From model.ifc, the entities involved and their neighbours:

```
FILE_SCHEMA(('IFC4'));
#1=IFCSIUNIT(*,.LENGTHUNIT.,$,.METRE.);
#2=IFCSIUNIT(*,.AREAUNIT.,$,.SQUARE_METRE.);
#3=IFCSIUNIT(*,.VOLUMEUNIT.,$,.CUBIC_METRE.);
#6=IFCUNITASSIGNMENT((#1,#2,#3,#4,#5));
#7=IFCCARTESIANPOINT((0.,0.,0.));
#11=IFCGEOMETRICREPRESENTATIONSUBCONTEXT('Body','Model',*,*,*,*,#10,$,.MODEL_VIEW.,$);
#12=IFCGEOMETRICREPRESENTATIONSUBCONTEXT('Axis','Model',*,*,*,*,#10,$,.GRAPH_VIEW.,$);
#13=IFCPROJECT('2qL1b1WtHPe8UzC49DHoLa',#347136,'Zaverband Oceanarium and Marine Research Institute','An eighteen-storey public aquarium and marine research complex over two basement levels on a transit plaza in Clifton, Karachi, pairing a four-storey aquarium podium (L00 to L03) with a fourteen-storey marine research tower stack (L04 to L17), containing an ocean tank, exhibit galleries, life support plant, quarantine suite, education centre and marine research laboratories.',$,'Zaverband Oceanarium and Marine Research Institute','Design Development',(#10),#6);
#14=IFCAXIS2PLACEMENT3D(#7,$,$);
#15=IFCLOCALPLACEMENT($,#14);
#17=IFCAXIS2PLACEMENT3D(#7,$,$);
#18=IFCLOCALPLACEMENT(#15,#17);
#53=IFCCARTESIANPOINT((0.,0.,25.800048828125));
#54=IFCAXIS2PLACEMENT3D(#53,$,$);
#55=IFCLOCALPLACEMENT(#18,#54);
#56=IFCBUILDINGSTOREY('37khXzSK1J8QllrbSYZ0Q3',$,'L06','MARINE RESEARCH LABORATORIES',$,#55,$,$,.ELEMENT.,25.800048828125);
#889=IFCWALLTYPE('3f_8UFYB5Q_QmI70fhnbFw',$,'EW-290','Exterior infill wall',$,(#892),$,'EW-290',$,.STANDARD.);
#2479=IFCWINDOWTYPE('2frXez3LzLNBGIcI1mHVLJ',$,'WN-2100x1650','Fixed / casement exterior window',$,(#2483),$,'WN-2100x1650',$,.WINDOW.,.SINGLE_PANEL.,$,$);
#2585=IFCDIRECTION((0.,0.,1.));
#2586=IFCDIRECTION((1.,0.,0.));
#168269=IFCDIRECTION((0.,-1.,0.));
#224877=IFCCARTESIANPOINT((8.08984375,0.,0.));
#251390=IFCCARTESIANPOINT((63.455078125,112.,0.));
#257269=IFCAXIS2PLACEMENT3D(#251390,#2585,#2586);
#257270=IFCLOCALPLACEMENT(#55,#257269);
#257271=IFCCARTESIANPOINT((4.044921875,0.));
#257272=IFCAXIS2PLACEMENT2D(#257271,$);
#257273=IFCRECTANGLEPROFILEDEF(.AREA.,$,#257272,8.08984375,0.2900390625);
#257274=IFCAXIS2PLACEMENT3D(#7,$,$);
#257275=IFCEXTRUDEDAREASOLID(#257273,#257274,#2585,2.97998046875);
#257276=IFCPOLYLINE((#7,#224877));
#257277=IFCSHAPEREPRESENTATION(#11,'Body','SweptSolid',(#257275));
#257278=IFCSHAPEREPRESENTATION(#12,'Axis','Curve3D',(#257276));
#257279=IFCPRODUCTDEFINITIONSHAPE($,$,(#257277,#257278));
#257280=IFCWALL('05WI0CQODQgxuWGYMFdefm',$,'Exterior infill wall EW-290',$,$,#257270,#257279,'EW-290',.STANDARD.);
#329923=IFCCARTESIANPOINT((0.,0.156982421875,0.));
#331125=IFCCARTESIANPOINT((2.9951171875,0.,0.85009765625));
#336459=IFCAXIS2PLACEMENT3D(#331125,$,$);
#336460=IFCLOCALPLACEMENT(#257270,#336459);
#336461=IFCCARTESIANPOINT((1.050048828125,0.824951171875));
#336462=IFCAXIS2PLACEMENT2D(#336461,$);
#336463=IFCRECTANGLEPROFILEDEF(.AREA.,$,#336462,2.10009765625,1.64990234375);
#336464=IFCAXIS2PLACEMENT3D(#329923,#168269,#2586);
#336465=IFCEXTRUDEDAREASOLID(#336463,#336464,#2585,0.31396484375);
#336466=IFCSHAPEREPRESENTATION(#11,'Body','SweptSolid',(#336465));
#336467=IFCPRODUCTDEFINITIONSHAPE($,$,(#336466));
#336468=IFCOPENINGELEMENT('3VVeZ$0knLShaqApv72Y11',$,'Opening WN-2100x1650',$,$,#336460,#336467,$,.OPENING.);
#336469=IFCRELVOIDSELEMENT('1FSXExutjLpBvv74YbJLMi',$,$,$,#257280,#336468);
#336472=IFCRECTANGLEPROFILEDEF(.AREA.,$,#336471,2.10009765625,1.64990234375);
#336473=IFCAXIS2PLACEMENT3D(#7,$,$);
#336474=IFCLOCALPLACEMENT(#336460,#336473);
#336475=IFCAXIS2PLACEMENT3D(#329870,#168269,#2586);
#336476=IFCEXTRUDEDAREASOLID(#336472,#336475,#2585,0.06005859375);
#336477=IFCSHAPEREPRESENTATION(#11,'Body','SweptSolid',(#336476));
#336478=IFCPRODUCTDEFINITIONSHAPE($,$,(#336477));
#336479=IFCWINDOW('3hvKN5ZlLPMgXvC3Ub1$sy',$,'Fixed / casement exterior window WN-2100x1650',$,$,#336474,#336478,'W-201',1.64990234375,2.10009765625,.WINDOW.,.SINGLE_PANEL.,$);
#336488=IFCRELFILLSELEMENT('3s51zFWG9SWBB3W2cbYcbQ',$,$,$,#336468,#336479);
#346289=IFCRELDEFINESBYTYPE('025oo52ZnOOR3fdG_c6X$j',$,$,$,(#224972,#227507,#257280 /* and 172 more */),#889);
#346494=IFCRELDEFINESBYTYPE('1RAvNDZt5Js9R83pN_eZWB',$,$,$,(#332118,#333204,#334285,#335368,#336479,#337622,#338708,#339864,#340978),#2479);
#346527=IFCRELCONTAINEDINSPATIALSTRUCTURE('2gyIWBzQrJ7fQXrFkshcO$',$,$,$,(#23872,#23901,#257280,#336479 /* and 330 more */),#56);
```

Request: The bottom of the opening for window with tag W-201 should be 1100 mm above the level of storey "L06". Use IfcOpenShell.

```python
import numpy as np
import ifcopenshell
import ifcopenshell.api.geometry
import ifcopenshell.geom
import ifcopenshell.util.element
import ifcopenshell.util.placement
import ifcopenshell.util.shape
import ifcopenshell.util.unit

model = ifcopenshell.open("model.ifc")
unit_scale = ifcopenshell.util.unit.calculate_unit_scale(model)

window = model.by_guid("3hvKN5ZlLPMgXvC3Ub1$sy")
opening = window.FillsVoids[0].RelatingOpeningElement
storey = ifcopenshell.util.element.get_container(window, ifc_class="IfcBuildingStorey")
level = ifcopenshell.util.placement.get_local_placement(storey.ObjectPlacement)[2, 3]

# The opening's origin need not be at the sill, so measure its lowest point.
shape = ifcopenshell.geom.create_shape(ifcopenshell.geom.settings(), opening)
bottom = ifcopenshell.util.shape.get_shape_bottom_elevation(shape, shape.geometry) / unit_scale
dz = level + 1.1 - bottom

shift = np.array([0.0, 0.0, dz])
# The window is placed relative to its opening, so it follows when the opening moves.
matrix = ifcopenshell.util.placement.get_local_placement(opening.ObjectPlacement)
matrix[:3, 3] += shift
ifcopenshell.api.geometry.edit_object_placement(
    model, product=opening, matrix=matrix, is_si=False, should_transform_children=True
)

print(f"moved by {dz * unit_scale:+.3f} m")

model.write("model_edited.ifc")
```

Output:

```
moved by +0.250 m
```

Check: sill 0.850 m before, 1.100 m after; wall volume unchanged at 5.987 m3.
